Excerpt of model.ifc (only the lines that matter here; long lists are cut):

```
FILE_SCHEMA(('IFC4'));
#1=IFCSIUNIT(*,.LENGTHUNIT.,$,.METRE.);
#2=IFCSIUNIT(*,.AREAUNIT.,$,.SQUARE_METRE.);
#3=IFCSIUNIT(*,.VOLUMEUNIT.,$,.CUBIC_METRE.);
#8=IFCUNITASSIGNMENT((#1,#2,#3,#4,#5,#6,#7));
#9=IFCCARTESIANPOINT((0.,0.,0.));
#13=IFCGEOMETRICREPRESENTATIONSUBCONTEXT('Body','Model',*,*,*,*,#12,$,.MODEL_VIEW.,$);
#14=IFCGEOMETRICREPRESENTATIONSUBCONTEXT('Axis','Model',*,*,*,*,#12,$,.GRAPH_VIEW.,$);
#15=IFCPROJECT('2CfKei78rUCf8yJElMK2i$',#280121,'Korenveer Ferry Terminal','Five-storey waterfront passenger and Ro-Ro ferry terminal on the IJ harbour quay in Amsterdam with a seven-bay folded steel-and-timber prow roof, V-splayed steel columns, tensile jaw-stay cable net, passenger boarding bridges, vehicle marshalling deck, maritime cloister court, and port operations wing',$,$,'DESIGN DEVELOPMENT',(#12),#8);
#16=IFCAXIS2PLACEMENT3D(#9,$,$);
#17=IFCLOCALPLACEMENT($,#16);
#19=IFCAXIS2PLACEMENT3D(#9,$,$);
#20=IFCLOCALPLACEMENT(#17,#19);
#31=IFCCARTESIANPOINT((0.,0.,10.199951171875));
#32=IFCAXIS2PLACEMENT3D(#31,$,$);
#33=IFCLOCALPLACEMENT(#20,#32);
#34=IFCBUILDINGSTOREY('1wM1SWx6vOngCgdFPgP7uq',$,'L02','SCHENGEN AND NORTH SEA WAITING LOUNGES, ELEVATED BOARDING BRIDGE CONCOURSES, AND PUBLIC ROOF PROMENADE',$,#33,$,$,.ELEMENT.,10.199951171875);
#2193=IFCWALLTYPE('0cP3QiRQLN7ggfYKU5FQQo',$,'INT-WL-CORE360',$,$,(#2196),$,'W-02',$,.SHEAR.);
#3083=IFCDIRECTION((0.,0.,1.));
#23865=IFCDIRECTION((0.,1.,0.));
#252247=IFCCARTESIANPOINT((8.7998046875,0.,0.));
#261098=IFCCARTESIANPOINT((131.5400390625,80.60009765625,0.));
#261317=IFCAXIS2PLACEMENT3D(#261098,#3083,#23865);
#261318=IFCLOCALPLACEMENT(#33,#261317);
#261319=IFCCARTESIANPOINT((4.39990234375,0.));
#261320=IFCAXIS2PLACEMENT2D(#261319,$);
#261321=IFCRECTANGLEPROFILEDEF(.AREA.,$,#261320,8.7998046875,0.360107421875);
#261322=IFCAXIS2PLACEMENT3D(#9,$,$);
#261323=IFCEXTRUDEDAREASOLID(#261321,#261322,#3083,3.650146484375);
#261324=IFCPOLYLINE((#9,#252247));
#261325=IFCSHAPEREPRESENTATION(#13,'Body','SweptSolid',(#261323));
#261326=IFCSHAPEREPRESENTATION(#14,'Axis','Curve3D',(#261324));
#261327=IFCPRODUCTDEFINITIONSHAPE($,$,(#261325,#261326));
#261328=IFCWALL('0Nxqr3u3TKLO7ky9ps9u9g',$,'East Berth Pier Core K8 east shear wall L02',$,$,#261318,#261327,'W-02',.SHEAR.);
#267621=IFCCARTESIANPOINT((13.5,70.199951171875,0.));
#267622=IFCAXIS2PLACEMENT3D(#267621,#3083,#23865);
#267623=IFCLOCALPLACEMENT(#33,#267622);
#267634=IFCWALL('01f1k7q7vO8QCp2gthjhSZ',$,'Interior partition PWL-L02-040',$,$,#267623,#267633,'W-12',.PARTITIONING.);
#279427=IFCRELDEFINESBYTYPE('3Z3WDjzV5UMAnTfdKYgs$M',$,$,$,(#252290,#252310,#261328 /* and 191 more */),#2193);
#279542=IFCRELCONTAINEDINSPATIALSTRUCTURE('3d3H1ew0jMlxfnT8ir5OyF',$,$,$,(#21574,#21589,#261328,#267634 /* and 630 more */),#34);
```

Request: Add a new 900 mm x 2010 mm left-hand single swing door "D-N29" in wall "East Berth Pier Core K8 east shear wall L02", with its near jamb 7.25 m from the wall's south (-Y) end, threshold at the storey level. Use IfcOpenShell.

```python
import numpy as np
import ifcopenshell
import ifcopenshell.api.feature
import ifcopenshell.api.geometry
import ifcopenshell.api.root
import ifcopenshell.api.spatial
import ifcopenshell.geom
import ifcopenshell.util.element
import ifcopenshell.util.placement
import ifcopenshell.util.representation
import ifcopenshell.util.shape
import ifcopenshell.util.unit

model = ifcopenshell.open("model.ifc")
unit_scale = ifcopenshell.util.unit.calculate_unit_scale(model)
settings = ifcopenshell.geom.settings()


def volume(element):
    """Net volume in cubic metres, openings subtracted."""
    shape = ifcopenshell.geom.create_shape(settings, element)
    return ifcopenshell.util.shape.get_volume(shape.geometry)


wall = model.by_guid("0Nxqr3u3TKLO7ky9ps9u9g")
storey = ifcopenshell.util.element.get_container(wall, ifc_class="IfcBuildingStorey")
context = ifcopenshell.util.representation.get_context(model, "Model", "Body", "MODEL_VIEW")
before = volume(wall)

width, height, from_end, sill = 0.9, 2.01, 7.25, 0.0  # metres

# The wall runs along its own X axis, and the end named is its -X end.
wall_shape = ifcopenshell.geom.create_shape(settings, wall)
x, y, z = ifcopenshell.util.shape.get_vertices(wall_shape.geometry).T
start = x.min() + from_end
face, thickness = float(y.min()), float(y.max() - y.min())
wall_matrix = ifcopenshell.util.placement.get_local_placement(wall.ObjectPlacement)
level = ifcopenshell.util.placement.get_local_placement(storey.ObjectPlacement)[2, 3]


def in_wall(x, y):
    """Placement at x, y metres in the wall's axes, at sill height."""
    matrix = wall_matrix.copy()
    matrix[:, 3] = wall_matrix @ np.array([x / unit_scale, y / unit_scale, 0.0, 1.0])
    matrix[2, 3] = level + sill / unit_scale
    return matrix


# Opening: a box that overshoots both wall faces by 50 mm.
opening = ifcopenshell.api.root.create_entity(model, ifc_class="IfcOpeningElement", predefined_type="OPENING")
box = ifcopenshell.api.geometry.add_wall_representation(
    model, context=context, length=width, height=height, thickness=thickness + 0.1
)
ifcopenshell.api.geometry.assign_representation(model, product=opening, representation=box)
ifcopenshell.api.geometry.edit_object_placement(model, product=opening, matrix=in_wall(start, face - 0.05), is_si=False)
ifcopenshell.api.feature.add_feature(model, feature=opening, element=wall)

door = ifcopenshell.api.root.create_entity(model, ifc_class="IfcDoor", name="D-N29", predefined_type="DOOR")
door.OverallWidth, door.OverallHeight = width / unit_scale, height / unit_scale
door.OperationType = "SINGLE_SWING_LEFT"
body = ifcopenshell.api.geometry.add_door_representation(
    model,
    context=context,
    overall_width=door.OverallWidth,
    overall_height=door.OverallHeight,
    operation_type="SINGLE_SWING_LEFT",
    lining_properties={"LiningDepth": thickness / unit_scale, "ThresholdDepth": thickness / unit_scale},
)
ifcopenshell.api.geometry.assign_representation(model, product=door, representation=body)
ifcopenshell.api.spatial.assign_container(model, products=[door], relating_structure=storey)
ifcopenshell.api.feature.add_filling(model, opening=opening, element=door)

# The lining spans the wall, so the door starts at the wall face.
ifcopenshell.api.geometry.edit_object_placement(model, product=door, matrix=in_wall(start, face), is_si=False)

after = volume(wall)

print(f"wall volume {before:.3f} -> {after:.3f} m3")

model.write("model_v2.ifc")
```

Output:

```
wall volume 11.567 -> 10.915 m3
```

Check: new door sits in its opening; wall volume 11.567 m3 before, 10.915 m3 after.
